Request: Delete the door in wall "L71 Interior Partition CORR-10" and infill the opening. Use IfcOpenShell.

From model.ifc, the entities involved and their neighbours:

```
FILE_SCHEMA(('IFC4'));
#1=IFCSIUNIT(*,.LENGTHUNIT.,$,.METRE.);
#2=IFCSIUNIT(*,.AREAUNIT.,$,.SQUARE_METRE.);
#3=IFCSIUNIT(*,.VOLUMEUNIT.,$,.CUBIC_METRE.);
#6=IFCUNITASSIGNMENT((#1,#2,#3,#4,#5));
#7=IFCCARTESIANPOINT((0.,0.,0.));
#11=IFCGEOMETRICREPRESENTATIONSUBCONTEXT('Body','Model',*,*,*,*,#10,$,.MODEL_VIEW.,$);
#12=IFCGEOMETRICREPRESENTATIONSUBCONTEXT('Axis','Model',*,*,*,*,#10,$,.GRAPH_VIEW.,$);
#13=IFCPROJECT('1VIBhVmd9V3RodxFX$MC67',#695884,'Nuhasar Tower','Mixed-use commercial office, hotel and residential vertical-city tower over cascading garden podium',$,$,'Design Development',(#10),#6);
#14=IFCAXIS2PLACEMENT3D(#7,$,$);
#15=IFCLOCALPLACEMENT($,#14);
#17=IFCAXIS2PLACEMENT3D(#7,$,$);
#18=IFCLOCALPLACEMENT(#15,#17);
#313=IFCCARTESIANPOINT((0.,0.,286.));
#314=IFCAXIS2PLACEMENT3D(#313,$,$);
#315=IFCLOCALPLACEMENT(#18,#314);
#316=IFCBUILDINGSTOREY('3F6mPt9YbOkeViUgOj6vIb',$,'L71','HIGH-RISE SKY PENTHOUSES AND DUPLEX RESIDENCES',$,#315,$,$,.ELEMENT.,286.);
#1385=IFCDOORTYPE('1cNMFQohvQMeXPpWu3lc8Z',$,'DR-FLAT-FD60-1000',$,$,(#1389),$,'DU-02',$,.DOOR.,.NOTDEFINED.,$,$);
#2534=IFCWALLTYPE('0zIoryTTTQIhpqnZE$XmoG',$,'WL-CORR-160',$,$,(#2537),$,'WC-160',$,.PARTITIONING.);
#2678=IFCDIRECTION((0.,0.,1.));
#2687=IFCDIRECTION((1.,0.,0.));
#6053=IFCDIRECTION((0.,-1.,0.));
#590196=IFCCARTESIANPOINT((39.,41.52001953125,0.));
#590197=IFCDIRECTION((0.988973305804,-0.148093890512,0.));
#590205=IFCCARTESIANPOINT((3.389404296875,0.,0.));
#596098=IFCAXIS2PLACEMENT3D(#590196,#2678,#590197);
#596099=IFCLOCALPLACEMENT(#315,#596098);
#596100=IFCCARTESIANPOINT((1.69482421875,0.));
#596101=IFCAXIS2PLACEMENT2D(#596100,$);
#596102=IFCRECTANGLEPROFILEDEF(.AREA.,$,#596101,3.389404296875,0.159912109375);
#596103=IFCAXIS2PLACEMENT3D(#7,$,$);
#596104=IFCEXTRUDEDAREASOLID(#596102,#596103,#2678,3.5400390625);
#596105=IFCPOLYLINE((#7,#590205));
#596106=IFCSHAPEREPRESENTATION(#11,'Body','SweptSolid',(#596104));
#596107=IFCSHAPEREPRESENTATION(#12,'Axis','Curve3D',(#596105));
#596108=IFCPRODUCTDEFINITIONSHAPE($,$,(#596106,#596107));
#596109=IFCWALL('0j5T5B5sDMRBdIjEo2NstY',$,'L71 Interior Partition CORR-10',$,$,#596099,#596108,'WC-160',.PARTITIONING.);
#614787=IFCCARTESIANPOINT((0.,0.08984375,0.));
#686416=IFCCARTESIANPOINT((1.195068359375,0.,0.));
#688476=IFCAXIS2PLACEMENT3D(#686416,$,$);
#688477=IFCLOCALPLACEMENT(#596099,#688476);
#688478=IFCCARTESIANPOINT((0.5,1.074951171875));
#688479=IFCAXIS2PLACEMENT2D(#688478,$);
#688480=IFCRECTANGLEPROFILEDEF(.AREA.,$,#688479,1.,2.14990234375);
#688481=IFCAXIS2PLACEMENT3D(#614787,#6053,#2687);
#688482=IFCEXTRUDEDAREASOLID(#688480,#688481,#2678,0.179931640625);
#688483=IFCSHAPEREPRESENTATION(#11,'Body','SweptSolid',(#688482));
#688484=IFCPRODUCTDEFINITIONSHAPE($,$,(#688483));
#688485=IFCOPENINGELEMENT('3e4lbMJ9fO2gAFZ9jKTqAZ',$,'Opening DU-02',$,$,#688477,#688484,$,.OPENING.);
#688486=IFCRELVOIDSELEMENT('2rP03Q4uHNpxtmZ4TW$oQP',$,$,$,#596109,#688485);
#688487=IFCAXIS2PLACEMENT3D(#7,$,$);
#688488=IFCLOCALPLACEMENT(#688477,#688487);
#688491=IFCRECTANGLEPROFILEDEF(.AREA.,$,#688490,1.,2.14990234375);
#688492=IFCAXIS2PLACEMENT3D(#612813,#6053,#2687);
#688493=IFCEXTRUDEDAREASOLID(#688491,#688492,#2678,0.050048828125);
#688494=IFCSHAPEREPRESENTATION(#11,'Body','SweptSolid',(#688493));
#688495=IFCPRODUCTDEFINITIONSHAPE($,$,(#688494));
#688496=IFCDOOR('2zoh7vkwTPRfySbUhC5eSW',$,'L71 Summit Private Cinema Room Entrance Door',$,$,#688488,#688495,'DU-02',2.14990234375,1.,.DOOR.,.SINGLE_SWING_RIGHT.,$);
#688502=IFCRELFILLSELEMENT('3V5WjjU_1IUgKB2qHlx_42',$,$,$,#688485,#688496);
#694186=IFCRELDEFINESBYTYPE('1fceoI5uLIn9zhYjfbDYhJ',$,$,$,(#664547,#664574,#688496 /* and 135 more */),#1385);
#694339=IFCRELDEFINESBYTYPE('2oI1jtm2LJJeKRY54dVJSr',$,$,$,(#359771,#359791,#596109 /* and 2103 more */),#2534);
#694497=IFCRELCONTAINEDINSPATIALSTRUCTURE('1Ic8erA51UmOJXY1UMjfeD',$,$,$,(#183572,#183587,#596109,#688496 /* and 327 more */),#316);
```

```python
import ifcopenshell
import ifcopenshell.api.feature
import ifcopenshell.api.root
import ifcopenshell.geom
import ifcopenshell.util.shape

model = ifcopenshell.open("model.ifc")
settings = ifcopenshell.geom.settings()


def volume(element):
    """Net volume in cubic metres, openings subtracted."""
    shape = ifcopenshell.geom.create_shape(settings, element)
    return ifcopenshell.util.shape.get_volume(shape.geometry)


door = model.by_id(688496)
opening = door.FillsVoids[0].RelatingOpeningElement
wall = opening.VoidsElements[0].RelatingBuildingElement
before = volume(wall)

ifcopenshell.api.root.remove_product(model, product=door)
ifcopenshell.api.feature.remove_feature(model, feature=opening)

after = volume(wall)

print(f"wall volume {before:.3f} -> {after:.3f} m3")

model.write("model-out.ifc")
```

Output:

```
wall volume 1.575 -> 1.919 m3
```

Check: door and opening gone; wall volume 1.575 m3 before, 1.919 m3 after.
